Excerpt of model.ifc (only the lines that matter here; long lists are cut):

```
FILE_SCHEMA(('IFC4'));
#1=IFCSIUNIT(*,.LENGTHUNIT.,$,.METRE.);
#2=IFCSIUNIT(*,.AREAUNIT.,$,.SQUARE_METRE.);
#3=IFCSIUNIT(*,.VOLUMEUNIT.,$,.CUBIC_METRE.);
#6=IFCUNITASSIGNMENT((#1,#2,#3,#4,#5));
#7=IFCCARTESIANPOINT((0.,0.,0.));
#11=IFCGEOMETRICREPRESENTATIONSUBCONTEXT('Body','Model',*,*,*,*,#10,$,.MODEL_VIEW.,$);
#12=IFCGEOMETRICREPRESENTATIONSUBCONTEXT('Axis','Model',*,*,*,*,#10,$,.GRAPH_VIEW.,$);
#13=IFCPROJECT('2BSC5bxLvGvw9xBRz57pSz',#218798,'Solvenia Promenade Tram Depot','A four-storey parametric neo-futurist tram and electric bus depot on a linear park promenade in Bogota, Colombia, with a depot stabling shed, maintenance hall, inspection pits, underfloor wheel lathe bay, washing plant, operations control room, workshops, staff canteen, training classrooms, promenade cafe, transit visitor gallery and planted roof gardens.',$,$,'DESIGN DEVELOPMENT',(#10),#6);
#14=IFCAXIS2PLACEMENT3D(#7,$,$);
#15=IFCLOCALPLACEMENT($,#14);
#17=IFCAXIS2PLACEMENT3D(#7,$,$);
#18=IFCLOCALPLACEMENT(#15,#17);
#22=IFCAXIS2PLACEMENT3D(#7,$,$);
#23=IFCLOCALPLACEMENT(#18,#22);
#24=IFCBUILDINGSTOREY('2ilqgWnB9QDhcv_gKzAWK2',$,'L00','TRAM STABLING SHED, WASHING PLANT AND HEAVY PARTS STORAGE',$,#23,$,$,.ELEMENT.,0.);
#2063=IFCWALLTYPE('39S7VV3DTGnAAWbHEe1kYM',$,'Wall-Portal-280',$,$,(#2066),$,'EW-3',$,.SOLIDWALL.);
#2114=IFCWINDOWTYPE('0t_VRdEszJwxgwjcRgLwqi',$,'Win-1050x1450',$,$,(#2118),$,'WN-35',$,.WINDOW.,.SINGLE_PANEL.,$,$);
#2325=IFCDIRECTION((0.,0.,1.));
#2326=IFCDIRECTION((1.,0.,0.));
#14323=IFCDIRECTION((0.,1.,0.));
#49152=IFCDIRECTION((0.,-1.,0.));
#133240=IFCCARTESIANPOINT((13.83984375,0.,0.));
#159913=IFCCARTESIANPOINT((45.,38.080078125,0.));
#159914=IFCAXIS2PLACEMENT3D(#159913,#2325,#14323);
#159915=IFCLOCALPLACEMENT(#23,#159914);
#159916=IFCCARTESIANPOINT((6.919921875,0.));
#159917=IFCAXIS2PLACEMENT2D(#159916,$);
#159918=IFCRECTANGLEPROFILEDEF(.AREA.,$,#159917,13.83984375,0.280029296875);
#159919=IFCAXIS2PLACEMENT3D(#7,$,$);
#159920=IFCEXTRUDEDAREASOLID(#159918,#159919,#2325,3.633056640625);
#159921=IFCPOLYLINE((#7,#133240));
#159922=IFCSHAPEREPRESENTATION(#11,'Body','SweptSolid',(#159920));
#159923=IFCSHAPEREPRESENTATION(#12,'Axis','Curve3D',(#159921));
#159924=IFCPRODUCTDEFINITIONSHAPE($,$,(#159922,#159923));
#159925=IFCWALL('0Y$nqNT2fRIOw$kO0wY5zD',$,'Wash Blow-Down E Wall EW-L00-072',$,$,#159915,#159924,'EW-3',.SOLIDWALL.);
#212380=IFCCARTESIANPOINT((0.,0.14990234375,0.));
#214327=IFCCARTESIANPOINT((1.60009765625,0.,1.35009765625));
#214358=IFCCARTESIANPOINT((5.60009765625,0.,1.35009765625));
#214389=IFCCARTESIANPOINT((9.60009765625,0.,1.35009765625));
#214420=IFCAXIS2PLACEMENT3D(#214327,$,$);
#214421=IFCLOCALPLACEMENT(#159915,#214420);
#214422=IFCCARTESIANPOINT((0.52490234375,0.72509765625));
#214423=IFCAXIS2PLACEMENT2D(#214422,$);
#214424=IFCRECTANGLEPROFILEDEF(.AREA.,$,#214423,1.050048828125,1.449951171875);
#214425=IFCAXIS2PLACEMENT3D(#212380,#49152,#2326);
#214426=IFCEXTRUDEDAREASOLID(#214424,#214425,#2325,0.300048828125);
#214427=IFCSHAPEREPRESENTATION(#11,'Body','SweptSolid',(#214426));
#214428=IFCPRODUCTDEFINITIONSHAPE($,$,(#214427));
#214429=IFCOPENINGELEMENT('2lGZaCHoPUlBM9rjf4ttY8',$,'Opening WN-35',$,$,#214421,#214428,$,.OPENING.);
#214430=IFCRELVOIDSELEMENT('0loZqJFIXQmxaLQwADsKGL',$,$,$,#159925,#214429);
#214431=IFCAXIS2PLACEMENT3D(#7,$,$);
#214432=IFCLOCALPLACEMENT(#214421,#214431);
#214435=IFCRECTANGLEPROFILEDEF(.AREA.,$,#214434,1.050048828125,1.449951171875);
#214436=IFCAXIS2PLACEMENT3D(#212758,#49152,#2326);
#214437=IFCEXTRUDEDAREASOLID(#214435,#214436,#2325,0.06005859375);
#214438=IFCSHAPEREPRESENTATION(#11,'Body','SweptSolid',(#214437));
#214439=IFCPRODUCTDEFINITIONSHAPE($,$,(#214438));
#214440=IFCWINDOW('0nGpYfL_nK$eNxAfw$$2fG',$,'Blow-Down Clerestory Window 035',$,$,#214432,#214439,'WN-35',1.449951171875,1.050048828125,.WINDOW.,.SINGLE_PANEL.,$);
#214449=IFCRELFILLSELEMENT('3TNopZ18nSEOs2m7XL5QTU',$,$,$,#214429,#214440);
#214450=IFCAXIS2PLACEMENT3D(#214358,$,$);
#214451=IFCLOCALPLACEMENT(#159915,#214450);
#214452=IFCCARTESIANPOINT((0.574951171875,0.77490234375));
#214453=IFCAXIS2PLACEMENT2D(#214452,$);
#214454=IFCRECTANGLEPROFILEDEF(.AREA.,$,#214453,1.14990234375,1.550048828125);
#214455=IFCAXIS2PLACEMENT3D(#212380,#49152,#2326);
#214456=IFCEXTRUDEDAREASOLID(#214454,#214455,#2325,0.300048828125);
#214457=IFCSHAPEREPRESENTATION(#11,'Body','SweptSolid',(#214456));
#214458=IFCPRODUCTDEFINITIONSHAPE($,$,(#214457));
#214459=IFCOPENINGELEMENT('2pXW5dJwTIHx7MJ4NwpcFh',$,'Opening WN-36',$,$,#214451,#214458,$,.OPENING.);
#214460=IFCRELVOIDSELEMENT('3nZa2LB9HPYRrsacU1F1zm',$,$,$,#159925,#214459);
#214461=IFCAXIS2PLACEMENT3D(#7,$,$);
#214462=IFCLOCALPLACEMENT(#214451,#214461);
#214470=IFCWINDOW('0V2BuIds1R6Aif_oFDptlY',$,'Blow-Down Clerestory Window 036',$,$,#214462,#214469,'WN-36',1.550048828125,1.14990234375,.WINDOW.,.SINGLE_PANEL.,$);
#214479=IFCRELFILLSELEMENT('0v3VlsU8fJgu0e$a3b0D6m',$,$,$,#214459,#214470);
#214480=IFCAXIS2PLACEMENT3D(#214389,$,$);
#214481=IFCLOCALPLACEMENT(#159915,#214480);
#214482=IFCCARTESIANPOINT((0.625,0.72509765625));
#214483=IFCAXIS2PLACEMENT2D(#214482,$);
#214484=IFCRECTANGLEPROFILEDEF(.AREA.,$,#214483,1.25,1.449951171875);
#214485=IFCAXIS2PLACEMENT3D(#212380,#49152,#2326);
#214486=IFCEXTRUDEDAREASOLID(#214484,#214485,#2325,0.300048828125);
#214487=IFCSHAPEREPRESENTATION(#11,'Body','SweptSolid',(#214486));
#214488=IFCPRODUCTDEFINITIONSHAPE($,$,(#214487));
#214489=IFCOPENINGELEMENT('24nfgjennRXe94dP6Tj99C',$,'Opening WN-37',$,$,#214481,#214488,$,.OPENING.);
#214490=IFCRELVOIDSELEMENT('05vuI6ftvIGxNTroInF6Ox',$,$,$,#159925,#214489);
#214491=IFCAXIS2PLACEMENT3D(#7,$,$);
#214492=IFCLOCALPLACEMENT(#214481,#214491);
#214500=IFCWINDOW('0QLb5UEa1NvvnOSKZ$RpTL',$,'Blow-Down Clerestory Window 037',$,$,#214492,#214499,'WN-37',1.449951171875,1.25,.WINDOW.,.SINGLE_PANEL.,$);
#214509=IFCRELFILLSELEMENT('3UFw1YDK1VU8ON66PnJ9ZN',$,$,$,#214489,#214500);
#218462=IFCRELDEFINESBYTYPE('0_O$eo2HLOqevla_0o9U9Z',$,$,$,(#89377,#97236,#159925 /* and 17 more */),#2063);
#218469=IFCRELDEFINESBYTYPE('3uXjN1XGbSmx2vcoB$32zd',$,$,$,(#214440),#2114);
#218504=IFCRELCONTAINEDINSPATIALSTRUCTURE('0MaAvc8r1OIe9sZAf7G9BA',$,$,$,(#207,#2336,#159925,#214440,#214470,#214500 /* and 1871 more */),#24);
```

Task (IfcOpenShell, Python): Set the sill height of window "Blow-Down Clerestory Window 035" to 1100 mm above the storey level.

```python
import numpy as np
import ifcopenshell
import ifcopenshell.api.geometry
import ifcopenshell.geom
import ifcopenshell.util.element
import ifcopenshell.util.placement
import ifcopenshell.util.shape
import ifcopenshell.util.unit

model = ifcopenshell.open("model.ifc")
unit_scale = ifcopenshell.util.unit.calculate_unit_scale(model)

window = model.by_guid("0nGpYfL_nK$eNxAfw$$2fG")
opening = window.FillsVoids[0].RelatingOpeningElement
storey = ifcopenshell.util.element.get_container(window, ifc_class="IfcBuildingStorey")
level = ifcopenshell.util.placement.get_local_placement(storey.ObjectPlacement)[2, 3]

# The opening's origin need not be at the sill, so measure its lowest point.
shape = ifcopenshell.geom.create_shape(ifcopenshell.geom.settings(), opening)
bottom = ifcopenshell.util.shape.get_shape_bottom_elevation(shape, shape.geometry) / unit_scale
dz = level + 1.1 / unit_scale - bottom

shift = np.array([0.0, 0.0, dz])
# The window is placed relative to its opening, so it follows when the opening moves.
matrix = ifcopenshell.util.placement.get_local_placement(opening.ObjectPlacement)
matrix[:3, 3] += shift
ifcopenshell.api.geometry.edit_object_placement(
    model, product=opening, matrix=matrix, is_si=False, should_transform_children=True
)

print(f"moved by {dz * unit_scale:+.3f} m")

model.write("model_rev.ifc")
```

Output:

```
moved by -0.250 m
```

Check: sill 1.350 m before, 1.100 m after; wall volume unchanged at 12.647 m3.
